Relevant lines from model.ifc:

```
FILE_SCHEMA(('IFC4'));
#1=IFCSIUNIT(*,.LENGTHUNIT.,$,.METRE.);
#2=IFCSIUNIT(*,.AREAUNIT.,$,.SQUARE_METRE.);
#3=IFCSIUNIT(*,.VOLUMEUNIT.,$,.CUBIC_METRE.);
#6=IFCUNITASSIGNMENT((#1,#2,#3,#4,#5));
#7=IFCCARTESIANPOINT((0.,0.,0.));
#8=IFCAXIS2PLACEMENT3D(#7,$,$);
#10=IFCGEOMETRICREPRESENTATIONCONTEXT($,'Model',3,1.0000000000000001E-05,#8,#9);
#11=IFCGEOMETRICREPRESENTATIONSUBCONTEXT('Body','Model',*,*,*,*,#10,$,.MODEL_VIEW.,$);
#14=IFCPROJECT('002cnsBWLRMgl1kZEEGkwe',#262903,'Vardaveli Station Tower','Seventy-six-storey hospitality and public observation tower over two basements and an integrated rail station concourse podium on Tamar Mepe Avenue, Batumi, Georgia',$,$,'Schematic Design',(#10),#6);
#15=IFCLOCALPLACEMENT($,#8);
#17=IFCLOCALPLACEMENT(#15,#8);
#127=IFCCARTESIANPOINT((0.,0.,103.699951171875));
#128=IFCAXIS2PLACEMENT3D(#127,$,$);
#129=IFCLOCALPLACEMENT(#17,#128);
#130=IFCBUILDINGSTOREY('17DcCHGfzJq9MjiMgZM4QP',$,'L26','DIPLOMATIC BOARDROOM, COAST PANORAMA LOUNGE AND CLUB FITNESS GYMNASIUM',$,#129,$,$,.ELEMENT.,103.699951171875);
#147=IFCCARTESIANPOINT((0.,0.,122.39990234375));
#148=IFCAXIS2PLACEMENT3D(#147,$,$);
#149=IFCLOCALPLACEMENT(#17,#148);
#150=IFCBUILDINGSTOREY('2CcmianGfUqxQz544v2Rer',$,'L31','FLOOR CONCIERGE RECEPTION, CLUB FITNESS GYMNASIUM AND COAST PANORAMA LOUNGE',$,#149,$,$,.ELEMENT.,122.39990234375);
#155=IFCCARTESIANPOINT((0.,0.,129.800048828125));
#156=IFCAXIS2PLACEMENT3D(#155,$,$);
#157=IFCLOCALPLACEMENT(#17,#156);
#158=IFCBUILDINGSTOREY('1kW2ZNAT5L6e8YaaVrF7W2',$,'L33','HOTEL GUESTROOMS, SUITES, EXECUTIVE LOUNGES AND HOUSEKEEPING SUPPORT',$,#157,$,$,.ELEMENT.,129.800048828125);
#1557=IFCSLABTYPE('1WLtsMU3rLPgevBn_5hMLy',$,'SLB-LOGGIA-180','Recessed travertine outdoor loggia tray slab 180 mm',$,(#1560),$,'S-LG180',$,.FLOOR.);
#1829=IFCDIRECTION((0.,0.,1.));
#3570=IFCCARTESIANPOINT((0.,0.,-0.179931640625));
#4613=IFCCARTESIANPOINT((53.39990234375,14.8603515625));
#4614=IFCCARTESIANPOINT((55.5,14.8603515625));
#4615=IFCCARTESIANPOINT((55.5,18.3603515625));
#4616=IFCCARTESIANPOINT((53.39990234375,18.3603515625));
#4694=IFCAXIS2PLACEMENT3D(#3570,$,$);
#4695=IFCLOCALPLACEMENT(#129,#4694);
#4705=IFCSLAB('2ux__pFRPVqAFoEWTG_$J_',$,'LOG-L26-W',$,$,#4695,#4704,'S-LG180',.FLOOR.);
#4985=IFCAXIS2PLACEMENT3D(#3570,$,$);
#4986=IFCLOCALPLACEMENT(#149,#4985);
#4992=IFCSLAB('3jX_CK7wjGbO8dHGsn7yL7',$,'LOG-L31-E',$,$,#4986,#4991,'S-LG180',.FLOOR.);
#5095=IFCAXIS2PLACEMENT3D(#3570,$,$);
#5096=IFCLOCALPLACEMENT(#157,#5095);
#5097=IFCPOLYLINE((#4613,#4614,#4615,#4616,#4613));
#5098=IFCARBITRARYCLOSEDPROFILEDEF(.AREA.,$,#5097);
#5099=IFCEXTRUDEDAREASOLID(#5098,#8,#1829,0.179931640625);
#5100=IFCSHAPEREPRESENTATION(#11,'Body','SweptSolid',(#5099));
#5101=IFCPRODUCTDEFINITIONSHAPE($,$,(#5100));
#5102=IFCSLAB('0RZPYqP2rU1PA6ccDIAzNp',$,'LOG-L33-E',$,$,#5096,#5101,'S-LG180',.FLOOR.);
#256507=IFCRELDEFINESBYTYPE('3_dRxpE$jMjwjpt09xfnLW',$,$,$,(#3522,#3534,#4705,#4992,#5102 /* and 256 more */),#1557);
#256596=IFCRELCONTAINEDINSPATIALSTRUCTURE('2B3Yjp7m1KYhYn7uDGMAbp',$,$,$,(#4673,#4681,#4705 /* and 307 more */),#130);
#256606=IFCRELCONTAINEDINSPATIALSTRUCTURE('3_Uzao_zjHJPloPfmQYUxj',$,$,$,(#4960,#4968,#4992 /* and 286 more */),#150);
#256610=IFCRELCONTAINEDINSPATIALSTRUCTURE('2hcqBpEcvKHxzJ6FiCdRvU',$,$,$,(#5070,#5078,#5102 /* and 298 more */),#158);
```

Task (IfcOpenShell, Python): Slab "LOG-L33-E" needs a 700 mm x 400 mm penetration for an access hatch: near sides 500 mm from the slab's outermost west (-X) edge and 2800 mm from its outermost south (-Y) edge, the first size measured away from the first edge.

```python
import numpy as np
import ifcopenshell
import ifcopenshell.api.feature
import ifcopenshell.api.geometry
import ifcopenshell.api.root
import ifcopenshell.geom
import ifcopenshell.util.placement
import ifcopenshell.util.representation
import ifcopenshell.util.shape
import ifcopenshell.util.unit

model = ifcopenshell.open("model.ifc")
unit_scale = ifcopenshell.util.unit.calculate_unit_scale(model)
settings = ifcopenshell.geom.settings()


def volume(element):
    """Net volume in cubic metres, openings subtracted."""
    shape = ifcopenshell.geom.create_shape(settings, element)
    return ifcopenshell.util.shape.get_volume(shape.geometry)


slab = model.by_guid("0RZPYqP2rU1PA6ccDIAzNp")
before = volume(slab)

# Extent in the slab's own axes, in metres. The edges named are its -X and -Y sides.
slab_shape = ifcopenshell.geom.create_shape(settings, slab)
vertices = ifcopenshell.util.shape.get_vertices(slab_shape.geometry)
x_min, y_min, bottom = vertices.min(axis=0)
top = vertices[:, 2].max()

opening = ifcopenshell.api.root.create_entity(model, ifc_class="IfcOpeningElement", name="Access hatch opening", predefined_type="OPENING")
context = ifcopenshell.util.representation.get_context(model, "Model", "Body", "MODEL_VIEW")
width, depth = 0.7, 0.4
outline = [(0.0, 0.0), (width, 0.0), (width, depth), (0.0, depth), (0.0, 0.0)]
# Overshoot both faces by 50 mm so the cut is clean.
shape = ifcopenshell.api.geometry.add_slab_representation(
    model, context=context, depth=top - bottom + 0.1, polyline=outline
)
ifcopenshell.api.geometry.assign_representation(model, product=opening, representation=shape)

matrix = ifcopenshell.util.placement.get_local_placement(slab.ObjectPlacement)
matrix[:, 3] = matrix @ np.append(np.array([x_min + 0.5, y_min + 2.8, bottom - 0.05]) / unit_scale, 1.0)
ifcopenshell.api.geometry.edit_object_placement(model, product=opening, matrix=matrix, is_si=False)
ifcopenshell.api.feature.add_feature(model, feature=opening, element=slab)

after = volume(slab)

print(f"slab volume {before:.3f} -> {after:.3f} m3")

model.write("model_v2.ifc")
```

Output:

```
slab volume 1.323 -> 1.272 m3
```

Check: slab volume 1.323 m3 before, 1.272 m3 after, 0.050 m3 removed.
